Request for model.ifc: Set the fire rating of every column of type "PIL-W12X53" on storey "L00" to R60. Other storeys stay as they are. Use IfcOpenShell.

First a look at what the model holds.

```python
import ifcopenshell
import ifcopenshell.util.element

model = ifcopenshell.open("model.ifc")
print(model.schema)
storey = next(s for s in model.by_type("IfcBuildingStorey") if s.Name == "L00")
columns = [e for e in ifcopenshell.util.element.get_decomposition(storey) if e.is_a("IfcColumn")]
seen = {}
for e in columns:
    element_type = ifcopenshell.util.element.get_type(e)
    key = (element_type.Name if element_type != e and element_type else None, ifcopenshell.util.element.get_pset(e, "Pset_ColumnCommon", "FireRating"))
    seen[key] = seen.get(key, 0) + 1
for (name, value), count in sorted(seen.items(), key=str):
    print(count, "x", name, "|", value)
```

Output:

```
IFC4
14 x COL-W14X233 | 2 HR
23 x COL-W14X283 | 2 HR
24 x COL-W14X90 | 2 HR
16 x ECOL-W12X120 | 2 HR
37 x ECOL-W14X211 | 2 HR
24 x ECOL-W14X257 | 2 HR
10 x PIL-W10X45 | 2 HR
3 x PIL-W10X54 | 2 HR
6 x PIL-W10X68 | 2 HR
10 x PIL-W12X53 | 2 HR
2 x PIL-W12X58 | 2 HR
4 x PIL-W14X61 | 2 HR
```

```python
import ifcopenshell
import ifcopenshell.api.pset
import ifcopenshell.util.element

model = ifcopenshell.open("model.ifc")

storey = next(s for s in model.by_type("IfcBuildingStorey") if s.Name == "L00")
columns = [e for e in ifcopenshell.util.element.get_decomposition(storey) if e.is_a("IfcColumn")]

count = 0
for e in columns:
    element_type = ifcopenshell.util.element.get_type(e)
    if element_type in (None, e) or element_type.Name != "PIL-W12X53":
        continue
    # add_pset returns the element's existing set when there is one.
    pset = ifcopenshell.api.pset.add_pset(model, product=e, name="Pset_ColumnCommon")
    ifcopenshell.api.pset.edit_pset(model, pset=pset, properties={"FireRating": "R60"})
    count += 1

print(count, "columns updated")

model.write("model-out.ifc")
```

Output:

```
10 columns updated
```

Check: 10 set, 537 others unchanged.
